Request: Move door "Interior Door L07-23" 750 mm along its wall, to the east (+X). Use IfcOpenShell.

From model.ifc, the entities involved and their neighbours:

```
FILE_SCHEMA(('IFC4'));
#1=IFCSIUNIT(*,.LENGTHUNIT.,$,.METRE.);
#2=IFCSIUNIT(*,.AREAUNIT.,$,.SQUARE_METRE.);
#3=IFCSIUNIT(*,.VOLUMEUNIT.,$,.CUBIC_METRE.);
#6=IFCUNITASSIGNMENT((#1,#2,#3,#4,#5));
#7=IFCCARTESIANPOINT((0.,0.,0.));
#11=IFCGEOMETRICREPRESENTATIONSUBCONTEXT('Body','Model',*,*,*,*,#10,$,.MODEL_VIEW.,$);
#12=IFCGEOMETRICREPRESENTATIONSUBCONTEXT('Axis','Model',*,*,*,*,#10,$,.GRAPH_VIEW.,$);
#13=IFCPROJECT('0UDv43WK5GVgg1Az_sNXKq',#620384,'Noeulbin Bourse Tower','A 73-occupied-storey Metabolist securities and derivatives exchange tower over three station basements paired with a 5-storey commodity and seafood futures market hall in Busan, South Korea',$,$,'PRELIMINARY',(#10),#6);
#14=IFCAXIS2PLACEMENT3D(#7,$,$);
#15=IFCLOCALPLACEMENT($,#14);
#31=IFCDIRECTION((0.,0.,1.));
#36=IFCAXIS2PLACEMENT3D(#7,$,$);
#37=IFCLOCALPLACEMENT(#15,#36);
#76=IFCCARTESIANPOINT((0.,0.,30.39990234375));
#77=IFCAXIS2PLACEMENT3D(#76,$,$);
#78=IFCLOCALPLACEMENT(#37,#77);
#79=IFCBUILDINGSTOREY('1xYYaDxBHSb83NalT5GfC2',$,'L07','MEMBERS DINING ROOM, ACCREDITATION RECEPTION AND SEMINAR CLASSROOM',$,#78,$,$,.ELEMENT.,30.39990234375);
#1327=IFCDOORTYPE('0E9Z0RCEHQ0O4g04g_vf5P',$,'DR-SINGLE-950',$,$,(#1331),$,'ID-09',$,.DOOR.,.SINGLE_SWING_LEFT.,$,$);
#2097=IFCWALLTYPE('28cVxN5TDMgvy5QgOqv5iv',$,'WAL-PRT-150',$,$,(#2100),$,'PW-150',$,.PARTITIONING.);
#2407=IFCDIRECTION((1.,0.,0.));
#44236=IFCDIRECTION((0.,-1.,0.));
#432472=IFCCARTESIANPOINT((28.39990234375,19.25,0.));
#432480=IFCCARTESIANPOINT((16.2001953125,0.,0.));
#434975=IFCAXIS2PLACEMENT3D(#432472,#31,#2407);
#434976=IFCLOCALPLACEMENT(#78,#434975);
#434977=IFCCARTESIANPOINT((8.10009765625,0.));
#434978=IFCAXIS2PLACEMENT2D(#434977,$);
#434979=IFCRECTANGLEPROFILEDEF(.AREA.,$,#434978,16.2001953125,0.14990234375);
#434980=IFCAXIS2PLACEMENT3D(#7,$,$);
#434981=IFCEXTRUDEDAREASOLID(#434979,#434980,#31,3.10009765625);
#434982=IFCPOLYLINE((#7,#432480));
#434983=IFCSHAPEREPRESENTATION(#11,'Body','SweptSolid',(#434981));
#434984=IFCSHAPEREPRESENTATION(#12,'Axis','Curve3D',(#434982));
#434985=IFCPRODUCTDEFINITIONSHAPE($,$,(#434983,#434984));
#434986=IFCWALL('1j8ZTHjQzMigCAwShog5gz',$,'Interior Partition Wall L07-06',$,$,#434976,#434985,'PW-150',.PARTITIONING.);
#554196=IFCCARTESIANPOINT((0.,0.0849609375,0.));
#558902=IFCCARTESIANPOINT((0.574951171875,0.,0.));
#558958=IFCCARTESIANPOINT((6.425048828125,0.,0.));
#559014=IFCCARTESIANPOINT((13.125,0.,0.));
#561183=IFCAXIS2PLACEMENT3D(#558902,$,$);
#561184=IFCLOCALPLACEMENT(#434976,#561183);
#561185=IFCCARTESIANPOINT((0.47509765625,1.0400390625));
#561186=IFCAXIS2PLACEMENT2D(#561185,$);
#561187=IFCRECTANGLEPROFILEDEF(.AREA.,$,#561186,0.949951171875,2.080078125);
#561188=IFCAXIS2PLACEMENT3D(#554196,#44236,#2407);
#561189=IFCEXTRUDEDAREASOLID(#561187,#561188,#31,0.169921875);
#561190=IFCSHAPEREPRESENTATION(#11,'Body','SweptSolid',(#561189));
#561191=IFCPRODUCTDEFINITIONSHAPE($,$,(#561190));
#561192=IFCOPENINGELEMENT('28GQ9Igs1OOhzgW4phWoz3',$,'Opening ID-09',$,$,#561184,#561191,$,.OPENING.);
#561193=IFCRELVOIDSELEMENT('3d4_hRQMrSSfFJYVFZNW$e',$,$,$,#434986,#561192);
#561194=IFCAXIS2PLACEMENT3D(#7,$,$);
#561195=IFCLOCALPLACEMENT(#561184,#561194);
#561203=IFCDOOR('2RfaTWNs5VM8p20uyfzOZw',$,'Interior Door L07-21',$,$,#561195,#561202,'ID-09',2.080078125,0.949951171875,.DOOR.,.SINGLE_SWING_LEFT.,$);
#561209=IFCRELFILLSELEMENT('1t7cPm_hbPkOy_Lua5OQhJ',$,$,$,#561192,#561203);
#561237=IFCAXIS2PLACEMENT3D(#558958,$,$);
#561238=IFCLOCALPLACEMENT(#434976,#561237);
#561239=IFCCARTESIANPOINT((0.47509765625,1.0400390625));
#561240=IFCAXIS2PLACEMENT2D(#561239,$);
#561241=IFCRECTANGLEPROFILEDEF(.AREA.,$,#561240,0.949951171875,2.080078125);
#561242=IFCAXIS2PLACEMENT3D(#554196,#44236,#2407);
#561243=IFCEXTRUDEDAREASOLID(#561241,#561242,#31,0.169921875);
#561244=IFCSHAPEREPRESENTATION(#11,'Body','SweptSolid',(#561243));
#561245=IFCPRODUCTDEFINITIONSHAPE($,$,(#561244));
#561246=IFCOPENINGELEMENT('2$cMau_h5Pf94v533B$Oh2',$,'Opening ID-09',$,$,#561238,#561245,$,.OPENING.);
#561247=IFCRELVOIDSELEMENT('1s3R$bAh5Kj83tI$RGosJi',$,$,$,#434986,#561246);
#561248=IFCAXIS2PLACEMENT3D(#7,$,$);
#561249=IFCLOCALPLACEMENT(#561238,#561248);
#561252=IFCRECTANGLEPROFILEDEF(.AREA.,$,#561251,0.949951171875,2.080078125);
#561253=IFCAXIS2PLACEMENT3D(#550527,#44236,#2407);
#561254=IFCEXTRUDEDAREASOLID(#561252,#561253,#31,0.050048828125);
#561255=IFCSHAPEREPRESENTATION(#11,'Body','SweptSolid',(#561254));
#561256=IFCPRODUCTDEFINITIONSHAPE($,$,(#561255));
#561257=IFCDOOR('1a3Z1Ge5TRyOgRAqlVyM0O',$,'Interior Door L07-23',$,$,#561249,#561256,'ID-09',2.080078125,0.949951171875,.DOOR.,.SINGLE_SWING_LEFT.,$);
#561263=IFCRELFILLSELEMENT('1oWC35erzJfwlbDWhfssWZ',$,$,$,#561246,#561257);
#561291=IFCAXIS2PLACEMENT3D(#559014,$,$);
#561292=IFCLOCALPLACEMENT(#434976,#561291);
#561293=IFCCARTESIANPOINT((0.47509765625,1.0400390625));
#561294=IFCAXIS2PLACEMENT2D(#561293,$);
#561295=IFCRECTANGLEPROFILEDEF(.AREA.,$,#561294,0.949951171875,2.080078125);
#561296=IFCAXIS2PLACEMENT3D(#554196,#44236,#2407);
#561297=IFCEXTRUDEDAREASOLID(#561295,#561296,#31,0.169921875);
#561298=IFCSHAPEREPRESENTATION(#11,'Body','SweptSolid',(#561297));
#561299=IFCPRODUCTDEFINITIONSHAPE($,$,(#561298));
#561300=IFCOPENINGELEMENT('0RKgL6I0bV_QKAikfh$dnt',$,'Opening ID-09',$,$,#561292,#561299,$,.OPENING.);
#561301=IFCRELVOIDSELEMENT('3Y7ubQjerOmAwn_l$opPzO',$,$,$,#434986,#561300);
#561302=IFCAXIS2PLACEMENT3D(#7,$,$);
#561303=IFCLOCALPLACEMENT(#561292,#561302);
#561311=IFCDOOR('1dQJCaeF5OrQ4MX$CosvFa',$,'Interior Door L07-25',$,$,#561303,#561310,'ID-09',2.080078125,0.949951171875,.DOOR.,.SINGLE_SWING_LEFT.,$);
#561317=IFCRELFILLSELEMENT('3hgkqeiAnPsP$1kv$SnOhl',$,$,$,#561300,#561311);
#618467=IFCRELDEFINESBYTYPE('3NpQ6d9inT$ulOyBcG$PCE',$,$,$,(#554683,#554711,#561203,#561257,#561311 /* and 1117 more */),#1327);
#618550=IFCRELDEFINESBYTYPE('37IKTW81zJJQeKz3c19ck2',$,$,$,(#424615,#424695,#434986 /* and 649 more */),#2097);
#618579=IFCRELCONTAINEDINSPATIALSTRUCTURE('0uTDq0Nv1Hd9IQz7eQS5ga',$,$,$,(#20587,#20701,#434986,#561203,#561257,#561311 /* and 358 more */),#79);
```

```python
import ifcopenshell
import ifcopenshell.api.geometry
import ifcopenshell.util.placement
import ifcopenshell.util.unit

model = ifcopenshell.open("model.ifc")
unit_scale = ifcopenshell.util.unit.calculate_unit_scale(model)

door = model.by_id(561257)
opening = door.FillsVoids[0].RelatingOpeningElement
wall = opening.VoidsElements[0].RelatingBuildingElement

wall_matrix = ifcopenshell.util.placement.get_local_placement(wall.ObjectPlacement)
shift = wall_matrix[:3, 0] * 0.75 / unit_scale
before = ifcopenshell.util.placement.get_local_placement(door.ObjectPlacement)[:3, 3].copy()

# The door is placed relative to its opening, so it follows when the opening moves.
matrix = ifcopenshell.util.placement.get_local_placement(opening.ObjectPlacement)
matrix[:3, 3] += shift
ifcopenshell.api.geometry.edit_object_placement(
    model, product=opening, matrix=matrix, is_si=False, should_transform_children=True
)

after = ifcopenshell.util.placement.get_local_placement(door.ObjectPlacement)[:3, 3]
print("door moved by", (after - before).round(3) + 0.0)

model.write("model-out.ifc")
```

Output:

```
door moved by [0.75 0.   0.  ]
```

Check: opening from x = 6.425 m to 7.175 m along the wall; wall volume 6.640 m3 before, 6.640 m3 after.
